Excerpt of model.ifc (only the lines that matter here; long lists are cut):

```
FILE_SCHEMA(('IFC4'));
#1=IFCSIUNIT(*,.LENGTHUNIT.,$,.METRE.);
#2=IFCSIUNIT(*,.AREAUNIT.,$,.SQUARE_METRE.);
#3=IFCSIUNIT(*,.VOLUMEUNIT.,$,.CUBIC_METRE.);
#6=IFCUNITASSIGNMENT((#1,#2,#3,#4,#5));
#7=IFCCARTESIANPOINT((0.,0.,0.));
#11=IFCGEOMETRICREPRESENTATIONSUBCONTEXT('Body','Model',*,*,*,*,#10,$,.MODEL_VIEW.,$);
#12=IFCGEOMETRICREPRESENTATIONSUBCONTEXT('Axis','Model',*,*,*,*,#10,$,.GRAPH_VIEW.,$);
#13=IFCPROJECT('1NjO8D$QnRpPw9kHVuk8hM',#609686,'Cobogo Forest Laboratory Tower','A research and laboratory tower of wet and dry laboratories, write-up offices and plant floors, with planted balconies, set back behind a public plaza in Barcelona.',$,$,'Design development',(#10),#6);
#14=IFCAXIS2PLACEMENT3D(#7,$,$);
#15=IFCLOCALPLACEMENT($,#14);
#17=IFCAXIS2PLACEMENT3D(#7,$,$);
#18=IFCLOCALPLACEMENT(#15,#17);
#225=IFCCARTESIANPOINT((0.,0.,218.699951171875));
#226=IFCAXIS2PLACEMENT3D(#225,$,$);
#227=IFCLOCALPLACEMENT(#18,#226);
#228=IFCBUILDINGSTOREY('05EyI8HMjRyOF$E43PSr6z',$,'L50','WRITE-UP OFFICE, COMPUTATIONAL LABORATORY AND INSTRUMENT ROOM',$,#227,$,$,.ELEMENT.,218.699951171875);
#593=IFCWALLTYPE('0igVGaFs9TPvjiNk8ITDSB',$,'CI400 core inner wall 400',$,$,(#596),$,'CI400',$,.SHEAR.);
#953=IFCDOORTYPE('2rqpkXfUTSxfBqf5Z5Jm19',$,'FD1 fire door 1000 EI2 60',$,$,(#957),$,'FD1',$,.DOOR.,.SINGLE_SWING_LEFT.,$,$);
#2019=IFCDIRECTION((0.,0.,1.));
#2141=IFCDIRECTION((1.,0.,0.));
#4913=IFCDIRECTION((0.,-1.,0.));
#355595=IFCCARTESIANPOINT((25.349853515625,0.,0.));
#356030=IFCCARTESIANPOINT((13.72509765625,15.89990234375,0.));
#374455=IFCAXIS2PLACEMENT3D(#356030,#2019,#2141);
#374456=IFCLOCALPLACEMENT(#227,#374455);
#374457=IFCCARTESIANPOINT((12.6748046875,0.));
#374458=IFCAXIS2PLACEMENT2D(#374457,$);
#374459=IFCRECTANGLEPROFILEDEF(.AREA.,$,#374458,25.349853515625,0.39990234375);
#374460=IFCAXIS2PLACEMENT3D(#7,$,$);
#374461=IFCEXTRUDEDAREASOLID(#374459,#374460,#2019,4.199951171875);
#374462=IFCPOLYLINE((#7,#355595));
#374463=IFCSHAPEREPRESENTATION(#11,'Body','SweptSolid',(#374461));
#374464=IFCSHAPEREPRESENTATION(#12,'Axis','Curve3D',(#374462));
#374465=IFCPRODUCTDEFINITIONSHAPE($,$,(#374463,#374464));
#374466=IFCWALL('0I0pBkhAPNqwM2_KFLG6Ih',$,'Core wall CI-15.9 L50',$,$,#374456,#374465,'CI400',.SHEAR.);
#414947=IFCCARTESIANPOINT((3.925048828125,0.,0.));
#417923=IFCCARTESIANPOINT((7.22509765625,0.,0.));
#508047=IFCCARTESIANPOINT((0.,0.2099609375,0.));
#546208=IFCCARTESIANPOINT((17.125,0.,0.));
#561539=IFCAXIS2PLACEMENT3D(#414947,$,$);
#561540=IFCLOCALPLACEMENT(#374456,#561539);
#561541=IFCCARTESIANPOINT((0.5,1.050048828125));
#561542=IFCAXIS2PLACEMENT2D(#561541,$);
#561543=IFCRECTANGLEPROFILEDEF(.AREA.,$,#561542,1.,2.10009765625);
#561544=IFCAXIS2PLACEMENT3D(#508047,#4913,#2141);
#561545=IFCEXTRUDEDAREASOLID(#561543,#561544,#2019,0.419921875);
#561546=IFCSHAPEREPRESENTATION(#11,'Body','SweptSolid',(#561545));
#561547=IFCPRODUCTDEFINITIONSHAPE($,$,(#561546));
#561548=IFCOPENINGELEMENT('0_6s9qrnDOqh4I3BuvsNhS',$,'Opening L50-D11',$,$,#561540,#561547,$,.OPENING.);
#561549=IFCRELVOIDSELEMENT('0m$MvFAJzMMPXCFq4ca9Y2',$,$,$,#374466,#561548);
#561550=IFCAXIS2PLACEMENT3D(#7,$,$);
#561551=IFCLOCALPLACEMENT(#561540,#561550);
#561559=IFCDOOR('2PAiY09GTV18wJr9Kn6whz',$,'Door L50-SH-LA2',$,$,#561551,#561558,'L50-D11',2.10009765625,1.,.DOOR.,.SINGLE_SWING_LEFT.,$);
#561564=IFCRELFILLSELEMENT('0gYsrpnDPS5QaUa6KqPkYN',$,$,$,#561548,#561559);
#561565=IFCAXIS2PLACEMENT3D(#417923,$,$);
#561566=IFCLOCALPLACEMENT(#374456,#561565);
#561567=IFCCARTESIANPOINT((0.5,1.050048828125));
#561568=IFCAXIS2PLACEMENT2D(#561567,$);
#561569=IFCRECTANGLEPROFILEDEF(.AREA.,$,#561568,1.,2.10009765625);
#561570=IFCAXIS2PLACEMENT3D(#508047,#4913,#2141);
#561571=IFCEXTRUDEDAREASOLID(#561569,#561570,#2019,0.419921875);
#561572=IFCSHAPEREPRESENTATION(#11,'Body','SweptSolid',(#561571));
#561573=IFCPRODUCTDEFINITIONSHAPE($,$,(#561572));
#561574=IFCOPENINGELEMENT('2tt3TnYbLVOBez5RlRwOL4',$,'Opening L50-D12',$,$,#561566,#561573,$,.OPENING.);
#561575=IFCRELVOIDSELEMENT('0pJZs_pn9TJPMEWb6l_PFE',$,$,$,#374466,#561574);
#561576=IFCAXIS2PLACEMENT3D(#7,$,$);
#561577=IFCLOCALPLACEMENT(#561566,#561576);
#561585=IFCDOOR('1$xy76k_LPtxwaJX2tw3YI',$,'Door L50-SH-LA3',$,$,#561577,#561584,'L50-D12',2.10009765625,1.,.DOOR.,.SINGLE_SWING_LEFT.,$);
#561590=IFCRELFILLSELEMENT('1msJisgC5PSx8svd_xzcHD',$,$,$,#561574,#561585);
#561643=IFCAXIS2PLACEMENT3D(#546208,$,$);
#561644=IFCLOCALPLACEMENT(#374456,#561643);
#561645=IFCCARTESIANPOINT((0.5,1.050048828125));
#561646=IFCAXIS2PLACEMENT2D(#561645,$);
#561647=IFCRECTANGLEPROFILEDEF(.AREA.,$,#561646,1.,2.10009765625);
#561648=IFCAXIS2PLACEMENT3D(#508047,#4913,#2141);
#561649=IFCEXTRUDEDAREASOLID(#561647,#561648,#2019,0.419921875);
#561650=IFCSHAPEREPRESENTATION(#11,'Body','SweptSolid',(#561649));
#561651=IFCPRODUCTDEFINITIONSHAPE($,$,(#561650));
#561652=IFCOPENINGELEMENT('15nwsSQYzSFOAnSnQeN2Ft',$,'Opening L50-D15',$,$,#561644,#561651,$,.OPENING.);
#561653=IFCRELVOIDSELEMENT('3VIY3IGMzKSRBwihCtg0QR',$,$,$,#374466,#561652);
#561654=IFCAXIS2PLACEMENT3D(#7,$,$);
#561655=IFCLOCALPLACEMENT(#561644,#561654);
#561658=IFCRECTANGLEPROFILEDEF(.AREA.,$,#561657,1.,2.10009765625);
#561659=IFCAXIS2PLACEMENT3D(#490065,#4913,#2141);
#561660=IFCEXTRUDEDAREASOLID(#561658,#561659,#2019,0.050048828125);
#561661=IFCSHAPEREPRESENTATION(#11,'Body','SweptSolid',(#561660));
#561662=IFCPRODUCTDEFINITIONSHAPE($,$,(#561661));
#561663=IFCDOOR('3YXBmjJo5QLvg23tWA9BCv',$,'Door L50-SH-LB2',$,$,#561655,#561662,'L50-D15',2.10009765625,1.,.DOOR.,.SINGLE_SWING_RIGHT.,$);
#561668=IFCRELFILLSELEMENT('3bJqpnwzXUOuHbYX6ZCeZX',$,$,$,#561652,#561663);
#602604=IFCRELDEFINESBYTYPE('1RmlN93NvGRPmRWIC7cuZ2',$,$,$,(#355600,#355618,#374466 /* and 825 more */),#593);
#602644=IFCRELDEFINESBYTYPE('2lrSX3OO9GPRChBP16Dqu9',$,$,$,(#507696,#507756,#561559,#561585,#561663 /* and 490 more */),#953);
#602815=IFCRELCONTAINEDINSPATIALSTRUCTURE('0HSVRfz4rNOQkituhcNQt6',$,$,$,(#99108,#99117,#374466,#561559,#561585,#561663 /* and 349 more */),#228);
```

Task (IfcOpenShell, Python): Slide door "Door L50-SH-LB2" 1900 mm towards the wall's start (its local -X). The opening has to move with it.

```python
import ifcopenshell
import ifcopenshell.api.geometry
import ifcopenshell.util.placement
import ifcopenshell.util.unit

model = ifcopenshell.open("model.ifc")
unit_scale = ifcopenshell.util.unit.calculate_unit_scale(model)

door = model.by_guid("3YXBmjJo5QLvg23tWA9BCv")
opening = door.FillsVoids[0].RelatingOpeningElement
wall = opening.VoidsElements[0].RelatingBuildingElement

wall_matrix = ifcopenshell.util.placement.get_local_placement(wall.ObjectPlacement)
shift = wall_matrix[:3, 0] * -1.9 / unit_scale
before = ifcopenshell.util.placement.get_local_placement(door.ObjectPlacement)[:3, 3].copy()

# The door is placed relative to its opening, so it follows when the opening moves.
matrix = ifcopenshell.util.placement.get_local_placement(opening.ObjectPlacement)
matrix[:3, 3] += shift
ifcopenshell.api.geometry.edit_object_placement(
    model, product=opening, matrix=matrix, is_si=False, should_transform_children=True
)

after = ifcopenshell.util.placement.get_local_placement(door.ObjectPlacement)[:3, 3]
print("door moved by", (after - before).round(3) + 0.0)

model.write("model_edited.ifc")
```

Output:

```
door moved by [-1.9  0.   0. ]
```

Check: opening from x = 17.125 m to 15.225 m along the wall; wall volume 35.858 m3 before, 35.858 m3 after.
